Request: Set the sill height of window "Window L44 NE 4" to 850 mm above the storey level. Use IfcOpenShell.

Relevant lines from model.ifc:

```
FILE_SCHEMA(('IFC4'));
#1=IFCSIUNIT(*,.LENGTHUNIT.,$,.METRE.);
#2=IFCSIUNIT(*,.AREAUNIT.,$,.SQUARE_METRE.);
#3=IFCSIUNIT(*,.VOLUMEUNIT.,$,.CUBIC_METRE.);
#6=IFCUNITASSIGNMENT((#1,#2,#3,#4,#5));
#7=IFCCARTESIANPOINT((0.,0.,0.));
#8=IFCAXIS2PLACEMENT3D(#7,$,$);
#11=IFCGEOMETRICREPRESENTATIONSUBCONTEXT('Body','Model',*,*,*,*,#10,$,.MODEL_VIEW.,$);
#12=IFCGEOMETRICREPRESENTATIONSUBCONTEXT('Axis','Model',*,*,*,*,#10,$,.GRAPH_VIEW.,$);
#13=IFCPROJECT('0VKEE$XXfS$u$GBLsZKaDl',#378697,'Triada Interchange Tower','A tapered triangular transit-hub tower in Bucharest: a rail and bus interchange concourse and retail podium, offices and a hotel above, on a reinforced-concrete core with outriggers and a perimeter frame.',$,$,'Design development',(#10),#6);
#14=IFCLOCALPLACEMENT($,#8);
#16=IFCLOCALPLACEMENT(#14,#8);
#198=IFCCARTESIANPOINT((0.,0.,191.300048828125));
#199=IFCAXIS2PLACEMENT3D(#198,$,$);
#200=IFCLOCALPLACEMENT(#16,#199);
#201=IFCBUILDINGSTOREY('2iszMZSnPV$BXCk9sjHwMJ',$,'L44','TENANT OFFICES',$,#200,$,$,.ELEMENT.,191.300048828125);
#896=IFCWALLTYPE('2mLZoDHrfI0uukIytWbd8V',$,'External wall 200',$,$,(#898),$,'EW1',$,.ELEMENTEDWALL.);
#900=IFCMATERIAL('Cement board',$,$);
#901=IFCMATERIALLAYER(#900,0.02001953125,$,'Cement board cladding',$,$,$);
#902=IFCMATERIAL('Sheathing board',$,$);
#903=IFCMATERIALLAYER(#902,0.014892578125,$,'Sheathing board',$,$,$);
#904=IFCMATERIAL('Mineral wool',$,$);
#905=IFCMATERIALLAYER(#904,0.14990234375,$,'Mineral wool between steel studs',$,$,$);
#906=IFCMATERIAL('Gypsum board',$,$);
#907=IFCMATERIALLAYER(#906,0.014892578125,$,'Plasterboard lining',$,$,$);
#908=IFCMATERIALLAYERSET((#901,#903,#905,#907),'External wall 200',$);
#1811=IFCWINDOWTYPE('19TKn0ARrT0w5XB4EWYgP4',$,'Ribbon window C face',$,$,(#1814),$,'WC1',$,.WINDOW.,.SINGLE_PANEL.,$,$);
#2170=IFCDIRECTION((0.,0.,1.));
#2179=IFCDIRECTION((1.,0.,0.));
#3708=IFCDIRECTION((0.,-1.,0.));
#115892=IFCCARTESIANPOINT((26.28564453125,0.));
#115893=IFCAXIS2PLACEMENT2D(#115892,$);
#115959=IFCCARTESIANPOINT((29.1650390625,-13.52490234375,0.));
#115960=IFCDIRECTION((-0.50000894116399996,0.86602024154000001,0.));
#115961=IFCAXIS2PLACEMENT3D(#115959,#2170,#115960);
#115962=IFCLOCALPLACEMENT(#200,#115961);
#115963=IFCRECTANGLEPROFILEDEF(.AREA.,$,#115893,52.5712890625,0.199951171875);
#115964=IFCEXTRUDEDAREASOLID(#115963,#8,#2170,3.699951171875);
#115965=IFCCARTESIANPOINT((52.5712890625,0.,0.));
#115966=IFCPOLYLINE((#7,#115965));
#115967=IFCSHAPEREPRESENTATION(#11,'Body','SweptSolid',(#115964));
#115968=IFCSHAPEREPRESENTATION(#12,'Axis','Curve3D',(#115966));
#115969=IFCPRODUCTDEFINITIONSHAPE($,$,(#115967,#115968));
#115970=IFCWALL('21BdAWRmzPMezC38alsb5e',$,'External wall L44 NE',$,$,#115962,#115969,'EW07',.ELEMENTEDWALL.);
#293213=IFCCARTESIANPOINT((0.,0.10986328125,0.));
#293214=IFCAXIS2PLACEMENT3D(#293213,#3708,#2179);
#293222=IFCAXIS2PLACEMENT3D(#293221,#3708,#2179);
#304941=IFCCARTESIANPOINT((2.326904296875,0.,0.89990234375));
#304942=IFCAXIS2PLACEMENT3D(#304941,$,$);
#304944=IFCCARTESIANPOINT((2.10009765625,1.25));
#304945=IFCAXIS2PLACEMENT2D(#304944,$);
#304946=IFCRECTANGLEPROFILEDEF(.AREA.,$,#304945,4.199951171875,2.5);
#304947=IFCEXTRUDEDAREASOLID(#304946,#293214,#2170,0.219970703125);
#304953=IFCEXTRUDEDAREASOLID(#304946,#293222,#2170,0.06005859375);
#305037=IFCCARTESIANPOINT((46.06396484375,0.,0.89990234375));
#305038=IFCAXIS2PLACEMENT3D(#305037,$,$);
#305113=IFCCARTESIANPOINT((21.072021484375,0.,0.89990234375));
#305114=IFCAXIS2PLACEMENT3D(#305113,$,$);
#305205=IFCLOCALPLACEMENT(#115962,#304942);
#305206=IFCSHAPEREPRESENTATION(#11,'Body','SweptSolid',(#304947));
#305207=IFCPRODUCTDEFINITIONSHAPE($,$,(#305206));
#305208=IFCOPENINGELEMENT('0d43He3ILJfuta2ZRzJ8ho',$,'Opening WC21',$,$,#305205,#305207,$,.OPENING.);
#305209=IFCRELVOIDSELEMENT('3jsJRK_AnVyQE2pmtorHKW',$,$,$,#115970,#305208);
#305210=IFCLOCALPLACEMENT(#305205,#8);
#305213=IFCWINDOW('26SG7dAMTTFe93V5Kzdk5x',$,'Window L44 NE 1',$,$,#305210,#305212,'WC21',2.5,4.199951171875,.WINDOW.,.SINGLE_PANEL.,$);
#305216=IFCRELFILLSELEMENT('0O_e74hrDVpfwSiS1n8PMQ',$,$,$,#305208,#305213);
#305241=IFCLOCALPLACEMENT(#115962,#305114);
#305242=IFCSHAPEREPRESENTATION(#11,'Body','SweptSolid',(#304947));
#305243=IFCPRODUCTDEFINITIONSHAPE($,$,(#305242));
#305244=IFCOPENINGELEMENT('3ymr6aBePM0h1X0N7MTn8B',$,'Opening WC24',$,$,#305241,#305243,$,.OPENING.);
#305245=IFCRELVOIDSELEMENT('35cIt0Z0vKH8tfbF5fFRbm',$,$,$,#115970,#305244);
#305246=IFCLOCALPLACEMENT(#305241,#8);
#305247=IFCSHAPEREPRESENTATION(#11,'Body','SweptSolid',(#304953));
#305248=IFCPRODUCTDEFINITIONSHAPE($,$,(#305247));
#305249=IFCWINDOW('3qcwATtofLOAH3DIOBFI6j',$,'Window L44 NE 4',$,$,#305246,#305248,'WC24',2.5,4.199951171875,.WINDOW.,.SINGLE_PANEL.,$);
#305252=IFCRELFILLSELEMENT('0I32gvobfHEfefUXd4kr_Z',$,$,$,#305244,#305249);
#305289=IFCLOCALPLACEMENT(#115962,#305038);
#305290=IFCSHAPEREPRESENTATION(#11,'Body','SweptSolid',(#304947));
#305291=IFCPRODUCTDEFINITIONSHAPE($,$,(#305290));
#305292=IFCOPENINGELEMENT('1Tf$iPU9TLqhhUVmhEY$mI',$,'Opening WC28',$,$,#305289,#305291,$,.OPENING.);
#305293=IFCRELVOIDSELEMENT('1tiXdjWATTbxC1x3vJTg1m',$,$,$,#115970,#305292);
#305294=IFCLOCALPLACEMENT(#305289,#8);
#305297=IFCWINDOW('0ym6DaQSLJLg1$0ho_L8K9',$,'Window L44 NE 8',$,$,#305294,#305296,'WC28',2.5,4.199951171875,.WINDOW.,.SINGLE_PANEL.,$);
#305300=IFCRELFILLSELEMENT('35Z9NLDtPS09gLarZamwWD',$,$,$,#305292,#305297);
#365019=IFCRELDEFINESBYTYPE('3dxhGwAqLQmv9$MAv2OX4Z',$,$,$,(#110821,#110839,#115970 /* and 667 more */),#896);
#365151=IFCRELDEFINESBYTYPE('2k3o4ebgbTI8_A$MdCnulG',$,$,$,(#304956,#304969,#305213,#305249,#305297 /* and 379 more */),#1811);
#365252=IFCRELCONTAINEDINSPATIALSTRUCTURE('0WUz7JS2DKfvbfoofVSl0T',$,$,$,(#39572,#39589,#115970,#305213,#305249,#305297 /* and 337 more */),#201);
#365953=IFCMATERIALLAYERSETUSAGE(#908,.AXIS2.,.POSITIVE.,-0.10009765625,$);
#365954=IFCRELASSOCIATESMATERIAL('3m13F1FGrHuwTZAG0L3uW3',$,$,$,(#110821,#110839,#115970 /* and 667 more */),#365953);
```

```python
import numpy as np
import ifcopenshell
import ifcopenshell.api.geometry
import ifcopenshell.geom
import ifcopenshell.util.element
import ifcopenshell.util.placement
import ifcopenshell.util.shape
import ifcopenshell.util.unit

model = ifcopenshell.open("model.ifc")
unit_scale = ifcopenshell.util.unit.calculate_unit_scale(model)

window = model.by_id(305249)
opening = window.FillsVoids[0].RelatingOpeningElement
storey = ifcopenshell.util.element.get_container(window, ifc_class="IfcBuildingStorey")
level = ifcopenshell.util.placement.get_local_placement(storey.ObjectPlacement)[2, 3]

# The opening's origin need not be at the sill, so measure its lowest point.
shape = ifcopenshell.geom.create_shape(ifcopenshell.geom.settings(), opening)
bottom = ifcopenshell.util.shape.get_shape_bottom_elevation(shape, shape.geometry) / unit_scale
dz = level + 0.85 - bottom

shift = np.array([0.0, 0.0, dz])
# The window is placed relative to its opening, so it follows when the opening moves.
matrix = ifcopenshell.util.placement.get_local_placement(opening.ObjectPlacement)
matrix[:3, 3] += shift
ifcopenshell.api.geometry.edit_object_placement(
    model, product=opening, matrix=matrix, is_si=False, should_transform_children=True
)

print(f"moved by {dz * unit_scale:+.3f} m")

model.write("model_rev.ifc")
```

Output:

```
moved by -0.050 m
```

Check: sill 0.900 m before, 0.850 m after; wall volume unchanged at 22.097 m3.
